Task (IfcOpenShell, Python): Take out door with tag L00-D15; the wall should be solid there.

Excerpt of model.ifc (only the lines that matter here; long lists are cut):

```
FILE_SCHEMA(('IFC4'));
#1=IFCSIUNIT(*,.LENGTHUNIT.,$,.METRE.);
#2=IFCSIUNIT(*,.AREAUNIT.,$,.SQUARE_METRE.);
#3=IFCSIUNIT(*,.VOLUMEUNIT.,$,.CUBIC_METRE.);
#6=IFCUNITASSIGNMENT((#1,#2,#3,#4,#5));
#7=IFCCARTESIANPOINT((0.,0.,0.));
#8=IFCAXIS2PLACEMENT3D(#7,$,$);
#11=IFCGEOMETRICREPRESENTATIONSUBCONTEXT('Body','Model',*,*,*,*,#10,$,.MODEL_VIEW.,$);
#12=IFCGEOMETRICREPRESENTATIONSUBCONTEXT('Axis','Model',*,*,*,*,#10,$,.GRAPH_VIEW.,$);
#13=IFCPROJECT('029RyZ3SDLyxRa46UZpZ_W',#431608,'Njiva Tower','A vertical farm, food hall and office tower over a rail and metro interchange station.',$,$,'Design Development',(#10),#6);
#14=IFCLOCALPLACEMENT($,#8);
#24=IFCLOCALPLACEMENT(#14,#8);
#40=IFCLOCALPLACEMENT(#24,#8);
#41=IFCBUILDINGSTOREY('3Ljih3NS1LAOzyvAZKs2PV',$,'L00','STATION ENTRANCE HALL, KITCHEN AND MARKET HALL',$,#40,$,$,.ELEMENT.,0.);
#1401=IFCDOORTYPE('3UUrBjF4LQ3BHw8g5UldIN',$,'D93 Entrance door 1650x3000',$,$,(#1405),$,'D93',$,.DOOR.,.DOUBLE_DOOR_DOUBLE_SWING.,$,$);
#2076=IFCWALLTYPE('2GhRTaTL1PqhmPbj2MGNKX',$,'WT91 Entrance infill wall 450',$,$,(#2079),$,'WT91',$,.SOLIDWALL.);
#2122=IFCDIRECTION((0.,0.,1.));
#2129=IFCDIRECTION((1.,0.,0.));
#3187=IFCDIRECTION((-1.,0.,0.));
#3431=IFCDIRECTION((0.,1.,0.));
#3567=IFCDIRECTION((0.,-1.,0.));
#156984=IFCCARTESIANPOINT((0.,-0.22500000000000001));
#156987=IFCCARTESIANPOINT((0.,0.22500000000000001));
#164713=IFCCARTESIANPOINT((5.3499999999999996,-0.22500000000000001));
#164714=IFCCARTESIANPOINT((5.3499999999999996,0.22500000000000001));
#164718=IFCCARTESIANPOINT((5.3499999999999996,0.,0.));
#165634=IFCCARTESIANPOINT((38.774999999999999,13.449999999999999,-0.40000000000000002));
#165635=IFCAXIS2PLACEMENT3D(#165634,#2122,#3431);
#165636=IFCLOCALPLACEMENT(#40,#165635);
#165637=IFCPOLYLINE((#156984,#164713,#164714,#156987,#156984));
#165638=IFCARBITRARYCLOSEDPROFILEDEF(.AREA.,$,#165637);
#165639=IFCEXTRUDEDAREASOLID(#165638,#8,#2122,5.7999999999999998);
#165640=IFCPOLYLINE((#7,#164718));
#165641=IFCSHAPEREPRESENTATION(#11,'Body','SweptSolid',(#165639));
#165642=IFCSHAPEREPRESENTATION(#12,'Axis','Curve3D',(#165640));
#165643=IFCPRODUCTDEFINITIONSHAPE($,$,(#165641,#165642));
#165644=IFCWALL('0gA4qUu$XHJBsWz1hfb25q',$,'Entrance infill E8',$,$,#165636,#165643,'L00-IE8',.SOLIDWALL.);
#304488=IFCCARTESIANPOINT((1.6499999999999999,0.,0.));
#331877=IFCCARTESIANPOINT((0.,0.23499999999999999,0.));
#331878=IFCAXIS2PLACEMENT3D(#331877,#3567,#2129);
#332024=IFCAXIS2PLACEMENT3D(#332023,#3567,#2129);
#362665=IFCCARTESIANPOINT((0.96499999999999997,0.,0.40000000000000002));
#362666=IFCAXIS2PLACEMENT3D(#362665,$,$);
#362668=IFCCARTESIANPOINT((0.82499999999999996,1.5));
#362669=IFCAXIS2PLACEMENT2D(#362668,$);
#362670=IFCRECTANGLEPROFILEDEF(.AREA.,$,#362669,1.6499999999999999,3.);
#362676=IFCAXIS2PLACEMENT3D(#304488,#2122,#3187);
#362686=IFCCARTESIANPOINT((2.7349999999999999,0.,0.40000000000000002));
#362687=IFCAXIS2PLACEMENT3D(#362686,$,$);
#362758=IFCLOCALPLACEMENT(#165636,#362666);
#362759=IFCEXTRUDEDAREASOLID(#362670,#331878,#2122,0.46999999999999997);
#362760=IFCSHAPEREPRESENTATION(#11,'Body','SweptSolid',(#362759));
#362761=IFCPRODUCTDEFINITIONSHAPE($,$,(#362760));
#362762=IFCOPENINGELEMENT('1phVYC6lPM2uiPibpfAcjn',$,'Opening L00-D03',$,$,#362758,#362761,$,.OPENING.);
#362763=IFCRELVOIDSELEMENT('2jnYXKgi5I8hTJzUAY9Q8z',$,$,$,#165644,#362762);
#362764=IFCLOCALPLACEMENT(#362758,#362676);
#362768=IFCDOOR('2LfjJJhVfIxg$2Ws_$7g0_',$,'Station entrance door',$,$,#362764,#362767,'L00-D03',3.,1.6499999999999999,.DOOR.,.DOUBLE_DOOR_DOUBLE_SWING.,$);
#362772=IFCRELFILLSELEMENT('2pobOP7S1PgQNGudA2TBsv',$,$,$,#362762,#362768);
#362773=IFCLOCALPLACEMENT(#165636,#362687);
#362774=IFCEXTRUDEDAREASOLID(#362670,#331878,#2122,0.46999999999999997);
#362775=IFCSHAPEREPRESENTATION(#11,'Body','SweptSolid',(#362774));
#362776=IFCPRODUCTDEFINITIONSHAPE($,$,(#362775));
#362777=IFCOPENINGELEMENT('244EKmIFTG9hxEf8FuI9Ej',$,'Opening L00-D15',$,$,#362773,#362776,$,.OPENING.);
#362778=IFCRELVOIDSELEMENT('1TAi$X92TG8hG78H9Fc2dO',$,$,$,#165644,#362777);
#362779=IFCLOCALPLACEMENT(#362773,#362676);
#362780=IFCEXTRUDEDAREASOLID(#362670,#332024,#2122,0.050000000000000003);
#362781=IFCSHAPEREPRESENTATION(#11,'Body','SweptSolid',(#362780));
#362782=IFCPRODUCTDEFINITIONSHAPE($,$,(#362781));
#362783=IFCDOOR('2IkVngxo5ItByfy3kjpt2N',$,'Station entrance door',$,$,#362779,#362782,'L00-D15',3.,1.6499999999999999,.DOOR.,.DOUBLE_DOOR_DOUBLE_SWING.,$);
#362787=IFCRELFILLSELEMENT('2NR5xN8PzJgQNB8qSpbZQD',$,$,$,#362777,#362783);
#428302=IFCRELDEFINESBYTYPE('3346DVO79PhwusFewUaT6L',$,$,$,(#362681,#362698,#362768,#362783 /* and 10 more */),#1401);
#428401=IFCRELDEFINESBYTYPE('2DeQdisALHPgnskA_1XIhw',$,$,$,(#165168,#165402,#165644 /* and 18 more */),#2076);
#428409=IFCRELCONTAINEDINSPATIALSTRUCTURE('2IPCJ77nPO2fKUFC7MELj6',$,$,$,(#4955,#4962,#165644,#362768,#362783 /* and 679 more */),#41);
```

```python
import ifcopenshell
import ifcopenshell.api.feature
import ifcopenshell.api.root
import ifcopenshell.geom
import ifcopenshell.util.shape

model = ifcopenshell.open("model.ifc")
settings = ifcopenshell.geom.settings()


def volume(element):
    """Net volume in cubic metres, openings subtracted."""
    shape = ifcopenshell.geom.create_shape(settings, element)
    return ifcopenshell.util.shape.get_volume(shape.geometry)


door = model.by_guid("2IkVngxo5ItByfy3kjpt2N")
opening = door.FillsVoids[0].RelatingOpeningElement
wall = opening.VoidsElements[0].RelatingBuildingElement
before = volume(wall)

ifcopenshell.api.root.remove_product(model, product=door)
ifcopenshell.api.feature.remove_feature(model, feature=opening)

after = volume(wall)

print(f"wall volume {before:.3f} -> {after:.3f} m3")

model.write("model-out.ifc")
```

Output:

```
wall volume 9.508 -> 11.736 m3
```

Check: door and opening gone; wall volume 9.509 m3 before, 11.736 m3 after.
